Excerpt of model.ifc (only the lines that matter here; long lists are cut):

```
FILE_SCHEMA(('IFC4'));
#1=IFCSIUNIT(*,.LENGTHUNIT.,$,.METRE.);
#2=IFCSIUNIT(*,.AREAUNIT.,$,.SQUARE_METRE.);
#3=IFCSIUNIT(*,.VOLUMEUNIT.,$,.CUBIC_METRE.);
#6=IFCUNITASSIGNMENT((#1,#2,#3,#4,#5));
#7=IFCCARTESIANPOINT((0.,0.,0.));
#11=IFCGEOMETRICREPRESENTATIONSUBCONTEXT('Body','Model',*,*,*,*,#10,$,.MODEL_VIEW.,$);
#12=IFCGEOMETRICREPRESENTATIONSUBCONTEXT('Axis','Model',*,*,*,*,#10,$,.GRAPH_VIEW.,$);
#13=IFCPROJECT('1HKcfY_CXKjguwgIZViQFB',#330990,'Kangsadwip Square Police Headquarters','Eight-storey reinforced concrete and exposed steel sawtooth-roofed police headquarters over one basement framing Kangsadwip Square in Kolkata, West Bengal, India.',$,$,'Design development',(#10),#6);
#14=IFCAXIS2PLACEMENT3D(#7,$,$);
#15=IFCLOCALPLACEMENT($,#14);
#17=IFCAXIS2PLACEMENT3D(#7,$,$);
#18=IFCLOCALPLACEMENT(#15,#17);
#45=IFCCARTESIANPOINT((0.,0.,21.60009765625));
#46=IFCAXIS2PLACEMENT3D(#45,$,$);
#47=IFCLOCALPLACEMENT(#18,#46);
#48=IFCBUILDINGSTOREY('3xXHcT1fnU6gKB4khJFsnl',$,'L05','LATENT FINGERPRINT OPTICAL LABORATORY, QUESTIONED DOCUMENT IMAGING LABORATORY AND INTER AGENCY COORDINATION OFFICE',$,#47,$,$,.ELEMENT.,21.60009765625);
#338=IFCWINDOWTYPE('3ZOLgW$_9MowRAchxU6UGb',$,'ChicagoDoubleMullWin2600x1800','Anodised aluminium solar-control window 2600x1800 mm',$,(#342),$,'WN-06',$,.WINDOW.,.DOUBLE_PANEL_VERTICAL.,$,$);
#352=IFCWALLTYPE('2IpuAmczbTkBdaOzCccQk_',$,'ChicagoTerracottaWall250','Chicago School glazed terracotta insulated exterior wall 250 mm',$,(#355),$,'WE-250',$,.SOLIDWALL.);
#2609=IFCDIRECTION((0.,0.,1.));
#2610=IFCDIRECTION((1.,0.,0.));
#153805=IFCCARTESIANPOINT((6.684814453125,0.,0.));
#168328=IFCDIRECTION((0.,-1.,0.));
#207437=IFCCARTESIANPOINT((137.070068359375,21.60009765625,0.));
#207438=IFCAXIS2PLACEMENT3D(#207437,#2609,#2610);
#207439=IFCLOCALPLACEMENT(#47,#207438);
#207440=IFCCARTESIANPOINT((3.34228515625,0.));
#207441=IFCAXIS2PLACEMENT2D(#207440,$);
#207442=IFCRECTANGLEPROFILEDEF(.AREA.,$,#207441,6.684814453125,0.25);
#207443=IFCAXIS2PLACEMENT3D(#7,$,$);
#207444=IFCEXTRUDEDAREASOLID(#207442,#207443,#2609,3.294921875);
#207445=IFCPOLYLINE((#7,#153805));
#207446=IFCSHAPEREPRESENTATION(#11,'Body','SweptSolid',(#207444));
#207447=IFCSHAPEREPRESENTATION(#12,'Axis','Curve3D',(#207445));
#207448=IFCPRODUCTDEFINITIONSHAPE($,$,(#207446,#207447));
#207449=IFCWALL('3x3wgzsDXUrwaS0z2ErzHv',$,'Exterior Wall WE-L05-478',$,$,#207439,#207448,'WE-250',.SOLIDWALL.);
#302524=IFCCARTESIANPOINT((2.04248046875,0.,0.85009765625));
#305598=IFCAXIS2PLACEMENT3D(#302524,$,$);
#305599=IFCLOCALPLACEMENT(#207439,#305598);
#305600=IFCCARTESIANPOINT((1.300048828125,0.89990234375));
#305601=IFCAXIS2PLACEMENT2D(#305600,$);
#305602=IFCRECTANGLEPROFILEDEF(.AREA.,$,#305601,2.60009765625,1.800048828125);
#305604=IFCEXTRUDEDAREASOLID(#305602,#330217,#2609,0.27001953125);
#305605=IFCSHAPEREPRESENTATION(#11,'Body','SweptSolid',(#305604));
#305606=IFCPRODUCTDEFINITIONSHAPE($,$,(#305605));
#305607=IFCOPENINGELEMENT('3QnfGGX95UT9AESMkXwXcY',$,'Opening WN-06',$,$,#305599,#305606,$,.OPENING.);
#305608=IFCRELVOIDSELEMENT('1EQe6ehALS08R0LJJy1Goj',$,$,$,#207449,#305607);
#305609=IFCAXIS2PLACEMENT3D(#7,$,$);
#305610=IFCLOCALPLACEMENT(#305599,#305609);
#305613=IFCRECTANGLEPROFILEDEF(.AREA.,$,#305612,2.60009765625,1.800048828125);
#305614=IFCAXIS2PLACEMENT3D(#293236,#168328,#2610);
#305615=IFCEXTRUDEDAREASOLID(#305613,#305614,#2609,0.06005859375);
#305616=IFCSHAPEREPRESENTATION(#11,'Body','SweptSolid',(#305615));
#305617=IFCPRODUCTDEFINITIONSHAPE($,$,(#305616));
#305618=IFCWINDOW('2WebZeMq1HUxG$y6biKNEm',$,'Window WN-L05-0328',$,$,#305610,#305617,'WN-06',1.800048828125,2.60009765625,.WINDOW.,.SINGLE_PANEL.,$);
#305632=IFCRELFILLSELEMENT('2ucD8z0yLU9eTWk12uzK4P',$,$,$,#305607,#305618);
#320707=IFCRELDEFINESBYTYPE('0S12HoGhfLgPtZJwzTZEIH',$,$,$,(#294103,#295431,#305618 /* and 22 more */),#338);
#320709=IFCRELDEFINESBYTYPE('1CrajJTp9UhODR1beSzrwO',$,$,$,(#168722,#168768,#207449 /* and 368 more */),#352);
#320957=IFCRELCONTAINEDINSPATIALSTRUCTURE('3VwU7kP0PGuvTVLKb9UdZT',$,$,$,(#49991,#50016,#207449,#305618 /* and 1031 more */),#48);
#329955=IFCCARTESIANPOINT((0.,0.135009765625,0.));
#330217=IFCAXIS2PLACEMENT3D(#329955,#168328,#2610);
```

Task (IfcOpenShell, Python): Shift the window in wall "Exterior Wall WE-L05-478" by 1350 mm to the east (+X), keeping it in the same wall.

```python
import ifcopenshell
import ifcopenshell.api.geometry
import ifcopenshell.util.placement

model = ifcopenshell.open("model.ifc")

window = model.by_guid("2WebZeMq1HUxG$y6biKNEm")
opening = window.FillsVoids[0].RelatingOpeningElement
wall = opening.VoidsElements[0].RelatingBuildingElement

wall_matrix = ifcopenshell.util.placement.get_local_placement(wall.ObjectPlacement)
shift = wall_matrix[:3, 0] * 1.35
before = ifcopenshell.util.placement.get_local_placement(window.ObjectPlacement)[:3, 3].copy()

# The window is placed relative to its opening, so it follows when the opening moves.
matrix = ifcopenshell.util.placement.get_local_placement(opening.ObjectPlacement)
matrix[:3, 3] += shift
ifcopenshell.api.geometry.edit_object_placement(
    model, product=opening, matrix=matrix, is_si=False, should_transform_children=True
)

after = ifcopenshell.util.placement.get_local_placement(window.ObjectPlacement)[:3, 3]
print("window moved by", (after - before).round(3) + 0.0)

model.write("model_edited.ifc")
```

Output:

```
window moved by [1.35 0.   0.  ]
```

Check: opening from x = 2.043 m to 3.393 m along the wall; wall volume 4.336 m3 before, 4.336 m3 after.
